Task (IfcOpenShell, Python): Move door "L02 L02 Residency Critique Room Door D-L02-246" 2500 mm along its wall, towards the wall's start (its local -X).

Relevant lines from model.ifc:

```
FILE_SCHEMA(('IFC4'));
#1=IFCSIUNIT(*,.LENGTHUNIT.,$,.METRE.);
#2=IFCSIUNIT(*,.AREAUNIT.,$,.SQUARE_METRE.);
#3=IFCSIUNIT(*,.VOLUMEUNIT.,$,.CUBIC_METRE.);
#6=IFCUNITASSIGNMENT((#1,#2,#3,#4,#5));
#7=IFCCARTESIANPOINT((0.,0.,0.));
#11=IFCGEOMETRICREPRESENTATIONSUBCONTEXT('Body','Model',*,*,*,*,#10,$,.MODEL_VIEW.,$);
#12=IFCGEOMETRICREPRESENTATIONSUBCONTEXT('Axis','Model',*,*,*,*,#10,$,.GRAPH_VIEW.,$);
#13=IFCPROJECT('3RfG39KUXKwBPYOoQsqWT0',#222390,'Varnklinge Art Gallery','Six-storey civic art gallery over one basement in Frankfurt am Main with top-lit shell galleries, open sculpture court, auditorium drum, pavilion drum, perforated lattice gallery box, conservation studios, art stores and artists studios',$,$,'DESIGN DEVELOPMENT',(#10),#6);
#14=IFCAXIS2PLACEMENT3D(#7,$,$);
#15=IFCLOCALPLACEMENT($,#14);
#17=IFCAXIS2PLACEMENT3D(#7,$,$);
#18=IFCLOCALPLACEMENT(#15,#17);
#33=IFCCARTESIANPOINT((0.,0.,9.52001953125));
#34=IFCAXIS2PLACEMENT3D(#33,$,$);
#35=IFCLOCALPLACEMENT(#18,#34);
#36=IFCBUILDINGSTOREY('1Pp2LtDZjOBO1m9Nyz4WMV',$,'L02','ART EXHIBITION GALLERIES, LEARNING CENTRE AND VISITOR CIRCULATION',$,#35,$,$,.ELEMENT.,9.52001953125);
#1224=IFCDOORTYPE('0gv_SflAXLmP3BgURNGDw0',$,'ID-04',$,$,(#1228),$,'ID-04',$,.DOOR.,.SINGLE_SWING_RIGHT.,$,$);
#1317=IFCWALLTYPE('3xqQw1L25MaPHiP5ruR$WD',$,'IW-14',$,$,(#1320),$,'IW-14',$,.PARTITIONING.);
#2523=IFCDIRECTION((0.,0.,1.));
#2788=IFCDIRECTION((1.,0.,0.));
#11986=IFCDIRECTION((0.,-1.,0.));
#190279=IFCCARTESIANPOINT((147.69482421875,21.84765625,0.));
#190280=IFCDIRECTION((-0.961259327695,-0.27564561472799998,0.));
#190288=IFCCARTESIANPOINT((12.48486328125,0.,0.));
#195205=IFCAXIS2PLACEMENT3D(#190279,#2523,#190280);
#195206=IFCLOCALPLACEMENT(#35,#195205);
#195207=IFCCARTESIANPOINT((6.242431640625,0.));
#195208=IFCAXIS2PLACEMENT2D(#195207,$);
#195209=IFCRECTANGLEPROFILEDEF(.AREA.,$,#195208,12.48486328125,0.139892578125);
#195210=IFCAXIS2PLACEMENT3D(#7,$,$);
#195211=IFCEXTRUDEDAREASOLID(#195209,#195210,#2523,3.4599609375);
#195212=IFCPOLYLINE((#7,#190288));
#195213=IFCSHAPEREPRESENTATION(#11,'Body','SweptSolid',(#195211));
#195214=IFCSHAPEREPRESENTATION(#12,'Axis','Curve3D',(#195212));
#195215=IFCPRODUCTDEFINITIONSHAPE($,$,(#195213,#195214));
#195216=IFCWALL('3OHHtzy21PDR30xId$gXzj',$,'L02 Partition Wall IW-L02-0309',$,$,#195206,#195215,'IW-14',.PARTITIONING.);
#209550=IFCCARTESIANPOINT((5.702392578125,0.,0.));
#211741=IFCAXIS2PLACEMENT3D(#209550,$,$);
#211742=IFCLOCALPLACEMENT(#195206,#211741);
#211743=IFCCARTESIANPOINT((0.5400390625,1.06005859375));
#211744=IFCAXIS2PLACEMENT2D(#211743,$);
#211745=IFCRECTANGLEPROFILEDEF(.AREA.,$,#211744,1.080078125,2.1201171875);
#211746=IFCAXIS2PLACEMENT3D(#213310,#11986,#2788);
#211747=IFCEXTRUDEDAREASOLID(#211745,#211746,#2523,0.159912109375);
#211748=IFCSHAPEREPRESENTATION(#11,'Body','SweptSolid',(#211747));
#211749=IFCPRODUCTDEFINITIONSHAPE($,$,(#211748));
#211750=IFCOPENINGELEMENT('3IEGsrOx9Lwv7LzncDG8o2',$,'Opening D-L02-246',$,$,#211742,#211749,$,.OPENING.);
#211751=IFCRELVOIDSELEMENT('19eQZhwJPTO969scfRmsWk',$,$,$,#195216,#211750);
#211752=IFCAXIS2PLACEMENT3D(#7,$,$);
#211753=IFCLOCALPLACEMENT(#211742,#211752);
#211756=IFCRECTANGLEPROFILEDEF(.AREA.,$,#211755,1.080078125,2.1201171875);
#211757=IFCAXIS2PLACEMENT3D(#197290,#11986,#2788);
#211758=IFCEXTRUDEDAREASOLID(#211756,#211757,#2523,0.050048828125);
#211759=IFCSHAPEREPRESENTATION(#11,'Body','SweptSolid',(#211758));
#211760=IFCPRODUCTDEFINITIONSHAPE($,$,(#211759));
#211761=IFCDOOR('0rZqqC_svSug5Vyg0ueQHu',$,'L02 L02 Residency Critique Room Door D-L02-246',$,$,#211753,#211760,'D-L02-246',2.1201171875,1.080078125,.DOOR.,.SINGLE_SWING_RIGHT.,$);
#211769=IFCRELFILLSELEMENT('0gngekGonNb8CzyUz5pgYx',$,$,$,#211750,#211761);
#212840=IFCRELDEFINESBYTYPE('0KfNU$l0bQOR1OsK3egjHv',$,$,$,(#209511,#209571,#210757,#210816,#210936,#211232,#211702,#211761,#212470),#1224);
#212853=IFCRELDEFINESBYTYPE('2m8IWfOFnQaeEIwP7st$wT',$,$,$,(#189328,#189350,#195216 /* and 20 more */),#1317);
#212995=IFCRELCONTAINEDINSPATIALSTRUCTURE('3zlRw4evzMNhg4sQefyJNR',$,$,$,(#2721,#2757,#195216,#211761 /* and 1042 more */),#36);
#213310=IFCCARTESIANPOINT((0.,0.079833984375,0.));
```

```python
import ifcopenshell
import ifcopenshell.api.geometry
import ifcopenshell.util.placement

model = ifcopenshell.open("model.ifc")

door = model.by_guid("0rZqqC_svSug5Vyg0ueQHu")
opening = door.FillsVoids[0].RelatingOpeningElement
wall = opening.VoidsElements[0].RelatingBuildingElement

wall_matrix = ifcopenshell.util.placement.get_local_placement(wall.ObjectPlacement)
shift = wall_matrix[:3, 0] * -2.5
before = ifcopenshell.util.placement.get_local_placement(door.ObjectPlacement)[:3, 3].copy()

# The door is placed relative to its opening, so it follows when the opening moves.
matrix = ifcopenshell.util.placement.get_local_placement(opening.ObjectPlacement)
matrix[:3, 3] += shift
ifcopenshell.api.geometry.edit_object_placement(
    model, product=opening, matrix=matrix, is_si=False, should_transform_children=True
)

after = ifcopenshell.util.placement.get_local_placement(door.ObjectPlacement)[:3, 3]
print("door moved by", (after - before).round(3) + 0.0)

model.write("model_edited.ifc")
```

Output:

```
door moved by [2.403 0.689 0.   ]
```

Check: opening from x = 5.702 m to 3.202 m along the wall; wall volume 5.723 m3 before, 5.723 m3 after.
